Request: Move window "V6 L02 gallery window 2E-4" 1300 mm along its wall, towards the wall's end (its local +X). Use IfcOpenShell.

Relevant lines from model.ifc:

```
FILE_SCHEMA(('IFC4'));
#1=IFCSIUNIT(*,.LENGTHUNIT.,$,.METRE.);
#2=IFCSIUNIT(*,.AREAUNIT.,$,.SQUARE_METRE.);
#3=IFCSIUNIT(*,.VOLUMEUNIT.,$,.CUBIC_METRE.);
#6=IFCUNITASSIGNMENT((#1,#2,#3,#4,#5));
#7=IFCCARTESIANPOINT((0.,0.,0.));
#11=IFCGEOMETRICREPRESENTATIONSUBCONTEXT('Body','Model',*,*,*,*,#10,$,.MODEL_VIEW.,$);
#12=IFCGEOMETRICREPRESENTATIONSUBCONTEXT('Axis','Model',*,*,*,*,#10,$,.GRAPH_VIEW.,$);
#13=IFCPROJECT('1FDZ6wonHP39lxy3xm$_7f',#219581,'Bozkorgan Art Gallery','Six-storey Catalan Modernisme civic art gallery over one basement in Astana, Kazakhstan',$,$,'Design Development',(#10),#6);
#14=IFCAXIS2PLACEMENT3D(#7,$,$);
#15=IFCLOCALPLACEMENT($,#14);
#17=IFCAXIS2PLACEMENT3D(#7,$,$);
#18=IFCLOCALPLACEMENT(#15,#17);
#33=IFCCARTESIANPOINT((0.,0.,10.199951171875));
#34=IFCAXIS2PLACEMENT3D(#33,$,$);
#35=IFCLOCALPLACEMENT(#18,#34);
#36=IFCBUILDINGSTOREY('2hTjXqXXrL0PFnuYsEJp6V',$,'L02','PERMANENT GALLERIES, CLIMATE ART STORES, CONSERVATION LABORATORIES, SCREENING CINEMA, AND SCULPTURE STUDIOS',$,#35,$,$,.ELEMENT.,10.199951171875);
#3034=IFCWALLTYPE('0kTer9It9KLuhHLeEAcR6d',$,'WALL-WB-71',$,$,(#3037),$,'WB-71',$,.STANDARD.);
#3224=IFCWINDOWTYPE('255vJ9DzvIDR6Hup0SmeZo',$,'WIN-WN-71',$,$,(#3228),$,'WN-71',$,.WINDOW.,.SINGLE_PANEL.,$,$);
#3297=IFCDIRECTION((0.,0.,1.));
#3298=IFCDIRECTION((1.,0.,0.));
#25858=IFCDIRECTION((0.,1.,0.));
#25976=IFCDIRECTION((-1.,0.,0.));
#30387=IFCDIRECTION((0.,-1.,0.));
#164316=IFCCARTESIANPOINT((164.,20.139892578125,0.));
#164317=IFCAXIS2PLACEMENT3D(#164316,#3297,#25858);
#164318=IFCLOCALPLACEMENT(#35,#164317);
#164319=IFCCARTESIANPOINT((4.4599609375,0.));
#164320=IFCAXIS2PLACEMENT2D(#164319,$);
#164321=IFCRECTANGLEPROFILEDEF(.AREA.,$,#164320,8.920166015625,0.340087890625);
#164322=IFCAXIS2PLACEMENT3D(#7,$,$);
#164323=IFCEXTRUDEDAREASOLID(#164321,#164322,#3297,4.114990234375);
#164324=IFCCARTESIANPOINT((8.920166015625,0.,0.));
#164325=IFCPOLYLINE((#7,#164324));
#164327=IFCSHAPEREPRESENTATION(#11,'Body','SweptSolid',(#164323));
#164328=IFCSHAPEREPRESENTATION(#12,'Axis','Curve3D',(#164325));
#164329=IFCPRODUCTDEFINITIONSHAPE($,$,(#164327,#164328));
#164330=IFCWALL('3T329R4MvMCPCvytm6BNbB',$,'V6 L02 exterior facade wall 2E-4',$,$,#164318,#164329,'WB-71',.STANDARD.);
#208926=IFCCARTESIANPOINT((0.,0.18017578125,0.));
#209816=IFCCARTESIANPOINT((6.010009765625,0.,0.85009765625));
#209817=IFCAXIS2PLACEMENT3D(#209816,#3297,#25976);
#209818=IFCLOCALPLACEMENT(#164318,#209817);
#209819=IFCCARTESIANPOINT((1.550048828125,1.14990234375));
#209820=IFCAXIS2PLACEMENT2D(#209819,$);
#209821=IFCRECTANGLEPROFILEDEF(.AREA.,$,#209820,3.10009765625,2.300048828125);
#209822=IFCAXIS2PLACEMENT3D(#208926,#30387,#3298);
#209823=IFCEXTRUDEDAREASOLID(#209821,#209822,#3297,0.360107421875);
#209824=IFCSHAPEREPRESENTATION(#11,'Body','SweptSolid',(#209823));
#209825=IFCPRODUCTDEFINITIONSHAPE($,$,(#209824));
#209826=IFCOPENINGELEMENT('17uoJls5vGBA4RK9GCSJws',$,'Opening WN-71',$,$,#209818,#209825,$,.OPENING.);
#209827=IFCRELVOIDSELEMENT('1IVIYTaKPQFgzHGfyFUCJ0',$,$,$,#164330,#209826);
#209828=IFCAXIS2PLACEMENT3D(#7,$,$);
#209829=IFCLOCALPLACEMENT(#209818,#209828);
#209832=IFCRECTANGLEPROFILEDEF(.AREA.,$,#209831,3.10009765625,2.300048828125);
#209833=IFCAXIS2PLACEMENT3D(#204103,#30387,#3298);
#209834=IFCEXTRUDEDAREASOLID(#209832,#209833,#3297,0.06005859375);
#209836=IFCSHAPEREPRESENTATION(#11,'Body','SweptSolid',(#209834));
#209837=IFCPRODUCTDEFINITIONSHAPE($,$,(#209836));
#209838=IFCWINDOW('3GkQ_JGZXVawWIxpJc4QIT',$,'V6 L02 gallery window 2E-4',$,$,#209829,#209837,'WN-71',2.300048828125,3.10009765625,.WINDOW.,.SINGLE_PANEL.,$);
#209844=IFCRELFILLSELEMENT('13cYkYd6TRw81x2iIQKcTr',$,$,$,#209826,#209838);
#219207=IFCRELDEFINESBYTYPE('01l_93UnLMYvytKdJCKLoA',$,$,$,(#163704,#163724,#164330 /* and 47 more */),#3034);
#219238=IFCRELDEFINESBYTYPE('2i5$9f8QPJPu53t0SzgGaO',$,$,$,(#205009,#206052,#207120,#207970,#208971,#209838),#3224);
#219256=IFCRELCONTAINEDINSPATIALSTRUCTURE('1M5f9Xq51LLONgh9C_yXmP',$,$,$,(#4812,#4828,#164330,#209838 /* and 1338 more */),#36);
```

```python
import ifcopenshell
import ifcopenshell.api.geometry
import ifcopenshell.util.placement

model = ifcopenshell.open("model.ifc")

window = model.by_guid("3GkQ_JGZXVawWIxpJc4QIT")
opening = window.FillsVoids[0].RelatingOpeningElement
wall = opening.VoidsElements[0].RelatingBuildingElement

wall_matrix = ifcopenshell.util.placement.get_local_placement(wall.ObjectPlacement)
shift = wall_matrix[:3, 0] * 1.3
before = ifcopenshell.util.placement.get_local_placement(window.ObjectPlacement)[:3, 3].copy()

# The window is placed relative to its opening, so it follows when the opening moves.
matrix = ifcopenshell.util.placement.get_local_placement(opening.ObjectPlacement)
matrix[:3, 3] += shift
ifcopenshell.api.geometry.edit_object_placement(
    model, product=opening, matrix=matrix, is_si=False, should_transform_children=True
)

after = ifcopenshell.util.placement.get_local_placement(window.ObjectPlacement)[:3, 3]
print("window moved by", (after - before).round(3) + 0.0)

model.write("model-out.ifc")
```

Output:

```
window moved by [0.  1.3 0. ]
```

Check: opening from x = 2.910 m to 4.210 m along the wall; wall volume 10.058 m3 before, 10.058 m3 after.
